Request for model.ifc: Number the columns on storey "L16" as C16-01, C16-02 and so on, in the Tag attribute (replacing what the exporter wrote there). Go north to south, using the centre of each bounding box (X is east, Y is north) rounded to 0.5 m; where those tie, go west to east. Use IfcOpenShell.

First a look at what the model holds.

```python
import ifcopenshell
import ifcopenshell.util.element
import ifcopenshell.util.placement

model = ifcopenshell.open("model.ifc")
print(model.schema)
storey = next(s for s in model.by_type("IfcBuildingStorey") if s.Name == "L16")
columns = [e for e in ifcopenshell.util.element.get_decomposition(storey) if e.is_a("IfcColumn")]
for e in sorted(columns, key=lambda e: e.id()):
    origin = ifcopenshell.util.placement.get_local_placement(e.ObjectPlacement)[:3, 3]
    print(e.id(), e.Tag, e.Name, origin.round(2) + 0.0, sep=" | ")
```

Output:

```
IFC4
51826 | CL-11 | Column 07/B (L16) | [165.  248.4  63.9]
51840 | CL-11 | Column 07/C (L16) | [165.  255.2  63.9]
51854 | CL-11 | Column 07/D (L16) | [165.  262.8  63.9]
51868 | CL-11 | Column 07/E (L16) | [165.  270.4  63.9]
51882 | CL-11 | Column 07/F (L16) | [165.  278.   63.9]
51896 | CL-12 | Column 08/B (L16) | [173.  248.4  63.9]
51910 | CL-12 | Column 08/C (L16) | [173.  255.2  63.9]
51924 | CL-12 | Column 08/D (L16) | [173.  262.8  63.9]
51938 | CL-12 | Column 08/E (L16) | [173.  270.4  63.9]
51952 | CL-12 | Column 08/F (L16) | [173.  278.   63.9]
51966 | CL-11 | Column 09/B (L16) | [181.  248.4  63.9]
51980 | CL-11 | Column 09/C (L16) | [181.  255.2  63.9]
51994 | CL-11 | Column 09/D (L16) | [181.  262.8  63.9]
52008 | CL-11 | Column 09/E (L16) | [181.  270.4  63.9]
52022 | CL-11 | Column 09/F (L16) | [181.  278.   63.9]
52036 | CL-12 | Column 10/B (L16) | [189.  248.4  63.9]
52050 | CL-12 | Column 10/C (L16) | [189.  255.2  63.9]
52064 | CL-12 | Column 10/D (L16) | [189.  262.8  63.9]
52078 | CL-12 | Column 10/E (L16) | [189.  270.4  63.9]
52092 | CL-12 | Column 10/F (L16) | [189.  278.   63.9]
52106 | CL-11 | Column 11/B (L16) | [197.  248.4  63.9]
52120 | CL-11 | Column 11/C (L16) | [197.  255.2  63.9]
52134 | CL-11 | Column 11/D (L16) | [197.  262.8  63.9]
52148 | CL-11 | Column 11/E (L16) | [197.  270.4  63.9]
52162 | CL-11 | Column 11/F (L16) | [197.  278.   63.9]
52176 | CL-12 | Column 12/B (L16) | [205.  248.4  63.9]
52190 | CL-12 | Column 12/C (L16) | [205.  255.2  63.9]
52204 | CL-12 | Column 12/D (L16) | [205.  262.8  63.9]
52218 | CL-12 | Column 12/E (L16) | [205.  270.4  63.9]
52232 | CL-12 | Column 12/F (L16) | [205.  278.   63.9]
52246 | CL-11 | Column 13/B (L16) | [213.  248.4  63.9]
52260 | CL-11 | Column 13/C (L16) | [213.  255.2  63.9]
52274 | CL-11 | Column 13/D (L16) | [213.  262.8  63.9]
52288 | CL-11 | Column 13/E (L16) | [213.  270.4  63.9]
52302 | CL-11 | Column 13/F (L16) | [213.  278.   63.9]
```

```python
import ifcopenshell
import ifcopenshell.geom
import ifcopenshell.util.element
import ifcopenshell.util.shape

model = ifcopenshell.open("model.ifc")
settings = ifcopenshell.geom.settings()
settings.set("use-world-coords", True)


def centre(element):
    shape = ifcopenshell.geom.create_shape(settings, element)
    return ifcopenshell.util.shape.get_bbox_centroid(shape.geometry)


storey = next(s for s in model.by_type("IfcBuildingStorey") if s.Name == "L16")
columns = [e for e in ifcopenshell.util.element.get_decomposition(storey) if e.is_a("IfcColumn")]

# Insertion points can sit at a corner or the storey origin, so sort by the geometry (in metres).
centres = {e: centre(e) for e in columns}
columns.sort(key=lambda e: (-round(centres[e][1] / 0.5), centres[e][0]))

for i, e in enumerate(columns, start=1):
    number = f"C16-{i:02d}"
    e.Tag = number
    print(e.id(), number)

model.write("model-out.ifc")
```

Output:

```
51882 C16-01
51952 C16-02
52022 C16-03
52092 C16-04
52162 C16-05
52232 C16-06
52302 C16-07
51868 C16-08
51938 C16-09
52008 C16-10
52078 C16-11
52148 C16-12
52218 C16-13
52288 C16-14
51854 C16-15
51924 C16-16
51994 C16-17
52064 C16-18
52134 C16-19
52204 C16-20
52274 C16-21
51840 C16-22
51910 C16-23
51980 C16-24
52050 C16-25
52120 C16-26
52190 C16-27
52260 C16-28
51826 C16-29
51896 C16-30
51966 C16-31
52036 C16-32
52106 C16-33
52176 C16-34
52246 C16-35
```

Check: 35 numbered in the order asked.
